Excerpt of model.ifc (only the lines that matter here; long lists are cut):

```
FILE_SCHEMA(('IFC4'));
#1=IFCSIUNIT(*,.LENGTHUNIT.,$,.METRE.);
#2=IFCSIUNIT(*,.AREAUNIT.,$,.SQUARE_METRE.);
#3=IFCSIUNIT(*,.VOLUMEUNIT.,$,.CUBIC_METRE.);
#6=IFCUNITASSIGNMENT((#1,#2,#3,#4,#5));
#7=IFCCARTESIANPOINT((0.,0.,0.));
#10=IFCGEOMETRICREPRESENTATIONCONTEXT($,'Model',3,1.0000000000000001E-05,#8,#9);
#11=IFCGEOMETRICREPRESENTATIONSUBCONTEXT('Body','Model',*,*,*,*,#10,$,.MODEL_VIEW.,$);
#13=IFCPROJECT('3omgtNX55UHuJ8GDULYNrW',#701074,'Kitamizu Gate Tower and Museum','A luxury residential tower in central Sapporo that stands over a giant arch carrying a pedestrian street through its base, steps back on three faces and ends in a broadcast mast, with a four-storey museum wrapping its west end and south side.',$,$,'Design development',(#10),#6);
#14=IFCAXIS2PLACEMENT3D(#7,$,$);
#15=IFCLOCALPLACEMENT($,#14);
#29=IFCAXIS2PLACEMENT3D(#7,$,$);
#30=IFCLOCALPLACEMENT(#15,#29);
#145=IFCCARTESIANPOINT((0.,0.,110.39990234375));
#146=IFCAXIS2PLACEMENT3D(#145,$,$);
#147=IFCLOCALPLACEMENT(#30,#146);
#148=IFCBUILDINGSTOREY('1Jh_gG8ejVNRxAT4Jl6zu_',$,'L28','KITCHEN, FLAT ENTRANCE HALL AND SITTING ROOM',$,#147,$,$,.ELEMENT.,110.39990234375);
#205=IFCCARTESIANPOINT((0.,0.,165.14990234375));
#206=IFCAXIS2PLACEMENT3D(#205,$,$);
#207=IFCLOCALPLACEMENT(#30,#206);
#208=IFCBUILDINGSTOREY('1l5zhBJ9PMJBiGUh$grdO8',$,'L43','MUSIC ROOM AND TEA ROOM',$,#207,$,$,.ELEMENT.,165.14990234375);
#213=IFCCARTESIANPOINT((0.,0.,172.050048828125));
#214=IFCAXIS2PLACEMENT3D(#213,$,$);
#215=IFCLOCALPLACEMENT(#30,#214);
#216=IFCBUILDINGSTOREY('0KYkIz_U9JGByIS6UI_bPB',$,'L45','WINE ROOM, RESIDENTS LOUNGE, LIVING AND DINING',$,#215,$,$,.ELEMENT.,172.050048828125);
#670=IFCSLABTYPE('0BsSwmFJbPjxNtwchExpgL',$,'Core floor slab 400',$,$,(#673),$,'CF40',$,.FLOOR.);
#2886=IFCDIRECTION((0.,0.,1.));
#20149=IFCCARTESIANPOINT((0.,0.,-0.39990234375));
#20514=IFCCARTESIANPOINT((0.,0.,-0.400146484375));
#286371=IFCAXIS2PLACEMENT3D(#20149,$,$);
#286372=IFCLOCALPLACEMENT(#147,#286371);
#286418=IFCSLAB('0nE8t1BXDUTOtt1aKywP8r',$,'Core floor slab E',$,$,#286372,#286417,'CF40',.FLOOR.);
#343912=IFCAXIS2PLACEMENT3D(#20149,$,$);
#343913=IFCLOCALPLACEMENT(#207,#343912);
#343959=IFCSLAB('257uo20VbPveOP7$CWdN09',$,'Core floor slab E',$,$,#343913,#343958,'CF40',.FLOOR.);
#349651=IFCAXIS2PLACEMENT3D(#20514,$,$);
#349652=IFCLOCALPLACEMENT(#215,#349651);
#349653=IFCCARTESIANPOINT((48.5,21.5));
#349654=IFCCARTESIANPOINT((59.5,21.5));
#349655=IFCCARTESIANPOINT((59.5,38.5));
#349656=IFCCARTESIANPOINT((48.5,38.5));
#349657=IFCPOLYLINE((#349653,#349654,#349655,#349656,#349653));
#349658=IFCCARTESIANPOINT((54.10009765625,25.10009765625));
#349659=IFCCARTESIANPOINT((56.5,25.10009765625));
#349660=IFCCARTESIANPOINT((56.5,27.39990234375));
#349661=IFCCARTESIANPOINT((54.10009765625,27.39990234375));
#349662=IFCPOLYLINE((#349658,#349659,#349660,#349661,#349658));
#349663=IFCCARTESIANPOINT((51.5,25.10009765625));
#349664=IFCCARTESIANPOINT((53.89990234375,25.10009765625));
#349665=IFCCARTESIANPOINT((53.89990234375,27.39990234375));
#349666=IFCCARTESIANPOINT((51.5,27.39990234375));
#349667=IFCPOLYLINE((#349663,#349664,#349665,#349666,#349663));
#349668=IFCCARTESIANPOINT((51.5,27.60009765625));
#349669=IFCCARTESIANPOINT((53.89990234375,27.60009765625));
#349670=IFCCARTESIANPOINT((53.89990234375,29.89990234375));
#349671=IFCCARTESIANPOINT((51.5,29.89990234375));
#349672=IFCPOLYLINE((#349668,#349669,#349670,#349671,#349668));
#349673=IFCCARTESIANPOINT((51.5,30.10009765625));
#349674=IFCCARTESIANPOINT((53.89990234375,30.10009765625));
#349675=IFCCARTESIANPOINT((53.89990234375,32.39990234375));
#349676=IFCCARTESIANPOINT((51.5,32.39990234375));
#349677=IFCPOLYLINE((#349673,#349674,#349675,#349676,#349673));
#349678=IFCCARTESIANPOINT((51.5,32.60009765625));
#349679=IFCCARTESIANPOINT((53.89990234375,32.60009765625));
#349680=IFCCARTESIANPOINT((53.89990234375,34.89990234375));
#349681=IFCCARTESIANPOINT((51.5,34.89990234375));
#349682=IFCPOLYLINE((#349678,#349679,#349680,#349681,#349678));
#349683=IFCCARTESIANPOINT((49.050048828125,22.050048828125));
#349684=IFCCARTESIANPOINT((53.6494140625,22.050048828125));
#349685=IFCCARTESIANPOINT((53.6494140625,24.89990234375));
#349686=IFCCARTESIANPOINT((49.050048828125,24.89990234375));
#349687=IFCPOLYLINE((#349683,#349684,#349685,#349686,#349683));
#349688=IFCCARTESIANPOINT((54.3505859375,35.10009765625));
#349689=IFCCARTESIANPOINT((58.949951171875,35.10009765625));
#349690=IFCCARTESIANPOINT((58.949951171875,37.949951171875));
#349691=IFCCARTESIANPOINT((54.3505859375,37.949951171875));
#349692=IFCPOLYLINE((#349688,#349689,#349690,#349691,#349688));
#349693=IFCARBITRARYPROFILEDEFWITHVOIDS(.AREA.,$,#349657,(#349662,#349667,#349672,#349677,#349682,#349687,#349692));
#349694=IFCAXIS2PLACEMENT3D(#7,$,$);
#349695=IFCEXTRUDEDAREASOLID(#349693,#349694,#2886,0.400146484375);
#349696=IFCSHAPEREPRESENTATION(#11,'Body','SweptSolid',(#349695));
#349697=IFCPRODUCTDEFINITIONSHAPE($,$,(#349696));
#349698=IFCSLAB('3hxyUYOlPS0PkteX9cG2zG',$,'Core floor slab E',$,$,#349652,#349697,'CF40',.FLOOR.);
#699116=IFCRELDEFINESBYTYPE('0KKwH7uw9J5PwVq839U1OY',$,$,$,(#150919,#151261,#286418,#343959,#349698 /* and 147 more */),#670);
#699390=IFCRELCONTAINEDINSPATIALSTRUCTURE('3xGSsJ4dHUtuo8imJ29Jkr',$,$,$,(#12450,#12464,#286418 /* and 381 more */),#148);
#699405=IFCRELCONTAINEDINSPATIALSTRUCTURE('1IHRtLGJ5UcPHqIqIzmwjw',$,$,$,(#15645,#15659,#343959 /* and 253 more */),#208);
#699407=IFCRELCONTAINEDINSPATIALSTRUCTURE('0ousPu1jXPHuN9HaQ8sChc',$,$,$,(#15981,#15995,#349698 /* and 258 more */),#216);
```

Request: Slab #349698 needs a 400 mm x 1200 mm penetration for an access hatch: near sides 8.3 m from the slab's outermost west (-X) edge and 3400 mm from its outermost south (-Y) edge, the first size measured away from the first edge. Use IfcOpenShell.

```python
import numpy as np
import ifcopenshell
import ifcopenshell.api.feature
import ifcopenshell.api.geometry
import ifcopenshell.api.root
import ifcopenshell.geom
import ifcopenshell.util.placement
import ifcopenshell.util.representation
import ifcopenshell.util.shape
import ifcopenshell.util.unit

model = ifcopenshell.open("model.ifc")
unit_scale = ifcopenshell.util.unit.calculate_unit_scale(model)
settings = ifcopenshell.geom.settings()


def volume(element):
    """Net volume in cubic metres, openings subtracted."""
    shape = ifcopenshell.geom.create_shape(settings, element)
    return ifcopenshell.util.shape.get_volume(shape.geometry)


slab = model.by_id(349698)
before = volume(slab)

# Extent in the slab's own axes, in metres. The edges named are its -X and -Y sides.
slab_shape = ifcopenshell.geom.create_shape(settings, slab)
vertices = ifcopenshell.util.shape.get_vertices(slab_shape.geometry)
x_min, y_min, bottom = vertices.min(axis=0)
top = vertices[:, 2].max()

opening = ifcopenshell.api.root.create_entity(model, ifc_class="IfcOpeningElement", name="Access hatch opening", predefined_type="OPENING")
context = ifcopenshell.util.representation.get_context(model, "Model", "Body", "MODEL_VIEW")
width, depth = 0.4, 1.2
outline = [(0.0, 0.0), (width, 0.0), (width, depth), (0.0, depth), (0.0, 0.0)]
# Overshoot both faces by 50 mm so the cut is clean.
shape = ifcopenshell.api.geometry.add_slab_representation(
    model, context=context, depth=top - bottom + 0.1, polyline=outline
)
ifcopenshell.api.geometry.assign_representation(model, product=opening, representation=shape)

matrix = ifcopenshell.util.placement.get_local_placement(slab.ObjectPlacement)
matrix[:, 3] = matrix @ np.append(np.array([x_min + 8.3, y_min + 3.4, bottom - 0.05]) / unit_scale, 1.0)
ifcopenshell.api.geometry.edit_object_placement(model, product=opening, matrix=matrix, is_si=False)
ifcopenshell.api.feature.add_feature(model, feature=opening, element=slab)

after = volume(slab)

print(f"slab volume {before:.3f} -> {after:.3f} m3")

model.write("model_edited.ifc")
```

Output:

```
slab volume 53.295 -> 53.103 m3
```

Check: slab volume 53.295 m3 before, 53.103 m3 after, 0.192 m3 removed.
